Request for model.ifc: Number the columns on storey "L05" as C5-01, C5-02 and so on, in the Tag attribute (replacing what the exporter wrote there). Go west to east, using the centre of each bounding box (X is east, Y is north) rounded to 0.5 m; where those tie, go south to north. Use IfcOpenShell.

First a look at what the model holds.

```python
import ifcopenshell
import ifcopenshell.util.element
import ifcopenshell.util.placement

model = ifcopenshell.open("model.ifc")
print(model.schema)
storey = next(s for s in model.by_type("IfcBuildingStorey") if s.Name == "L05")
columns = [e for e in ifcopenshell.util.element.get_decomposition(storey) if e.is_a("IfcColumn")]
for e in sorted(columns, key=lambda e: e.id()):
    origin = ifcopenshell.util.placement.get_local_placement(e.ObjectPlacement)[:3, 3]
    print(e.id(), e.Tag, e.Name, origin.round(2) + 0.0, sep=" | ")
```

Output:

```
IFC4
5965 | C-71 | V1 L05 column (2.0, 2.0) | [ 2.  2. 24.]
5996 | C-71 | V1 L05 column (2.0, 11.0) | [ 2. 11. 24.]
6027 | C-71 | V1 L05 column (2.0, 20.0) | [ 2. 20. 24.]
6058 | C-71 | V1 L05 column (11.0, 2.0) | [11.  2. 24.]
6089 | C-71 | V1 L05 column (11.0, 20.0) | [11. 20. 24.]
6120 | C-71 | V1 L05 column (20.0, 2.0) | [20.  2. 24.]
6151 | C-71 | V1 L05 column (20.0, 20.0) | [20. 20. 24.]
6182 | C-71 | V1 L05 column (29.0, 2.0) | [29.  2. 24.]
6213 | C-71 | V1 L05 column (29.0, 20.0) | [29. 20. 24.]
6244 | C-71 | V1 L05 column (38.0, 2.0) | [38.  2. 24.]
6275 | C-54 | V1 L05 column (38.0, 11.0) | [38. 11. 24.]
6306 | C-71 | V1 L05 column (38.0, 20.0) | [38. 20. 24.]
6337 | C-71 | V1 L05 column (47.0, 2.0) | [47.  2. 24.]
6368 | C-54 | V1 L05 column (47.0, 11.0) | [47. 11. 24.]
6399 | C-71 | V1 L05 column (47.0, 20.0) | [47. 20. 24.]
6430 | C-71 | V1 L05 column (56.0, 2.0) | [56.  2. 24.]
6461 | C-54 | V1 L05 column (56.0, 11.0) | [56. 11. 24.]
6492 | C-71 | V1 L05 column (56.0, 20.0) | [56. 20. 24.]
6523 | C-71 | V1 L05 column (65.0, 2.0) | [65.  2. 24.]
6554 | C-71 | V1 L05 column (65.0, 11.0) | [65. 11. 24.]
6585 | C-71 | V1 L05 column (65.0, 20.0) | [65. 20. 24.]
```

```python
import ifcopenshell
import ifcopenshell.geom
import ifcopenshell.util.element
import ifcopenshell.util.shape

model = ifcopenshell.open("model.ifc")
settings = ifcopenshell.geom.settings()
settings.set("use-world-coords", True)


def centre(element):
    shape = ifcopenshell.geom.create_shape(settings, element)
    return ifcopenshell.util.shape.get_bbox_centroid(shape.geometry)


storey = next(s for s in model.by_type("IfcBuildingStorey") if s.Name == "L05")
columns = [e for e in ifcopenshell.util.element.get_decomposition(storey) if e.is_a("IfcColumn")]

# Insertion points can sit at a corner or the storey origin, so sort by the geometry (in metres).
centres = {e: centre(e) for e in columns}
columns.sort(key=lambda e: (round(centres[e][0] / 0.5), centres[e][1]))

for i, e in enumerate(columns, start=1):
    number = f"C5-{i:02d}"
    e.Tag = number
    print(e.id(), number)

model.write("model_v2.ifc")
```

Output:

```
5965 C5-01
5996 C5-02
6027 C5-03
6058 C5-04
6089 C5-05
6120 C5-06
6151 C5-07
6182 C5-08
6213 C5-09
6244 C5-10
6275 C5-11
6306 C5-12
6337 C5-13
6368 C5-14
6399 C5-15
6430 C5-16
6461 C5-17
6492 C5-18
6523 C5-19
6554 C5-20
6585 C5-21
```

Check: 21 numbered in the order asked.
